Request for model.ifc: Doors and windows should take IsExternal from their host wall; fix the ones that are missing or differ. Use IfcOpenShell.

First a look at what the model holds.

```python
import ifcopenshell
import ifcopenshell.util.element

model = ifcopenshell.open("model.ifc")
print(model.schema)
seen = {}
for e in model.by_type("IfcDoor") + model.by_type("IfcWindow"):
    if not e.FillsVoids:
        continue
    host = e.FillsVoids[0].RelatingOpeningElement.VoidsElements[0].RelatingBuildingElement
    own = ifcopenshell.util.element.get_pset(e, f"Pset_{e.is_a()[3:].removesuffix('StandardCase')}Common", "IsExternal")
    wall = ifcopenshell.util.element.get_pset(host, "Pset_WallCommon", "IsExternal")
    seen[e.is_a(), own, wall] = seen.get((e.is_a(), own, wall), 0) + 1
for (cls, own, wall), count in sorted(seen.items(), key=str):
    print(count, cls, "IsExternal:", own, "| host wall:", wall)
```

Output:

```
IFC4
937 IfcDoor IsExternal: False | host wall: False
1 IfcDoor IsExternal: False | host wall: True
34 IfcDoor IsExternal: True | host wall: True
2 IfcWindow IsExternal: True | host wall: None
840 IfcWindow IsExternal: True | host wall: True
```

```python
import ifcopenshell
import ifcopenshell.api.pset
import ifcopenshell.util.element

model = ifcopenshell.open("model.ifc")

count = 0
for ifc_class, pset_name in (("IfcDoor", "Pset_DoorCommon"), ("IfcWindow", "Pset_WindowCommon")):
    for e in model.by_type(ifc_class):
        if not e.FillsVoids:
            continue
        host = e.FillsVoids[0].RelatingOpeningElement.VoidsElements[0].RelatingBuildingElement
        external = ifcopenshell.util.element.get_pset(host, "Pset_WallCommon", "IsExternal")
        if external is None or ifcopenshell.util.element.get_pset(e, pset_name, "IsExternal") == external:
            continue
        pset = ifcopenshell.api.pset.add_pset(model, product=e, name=pset_name)
        ifcopenshell.api.pset.edit_pset(model, pset=pset, properties={"IsExternal": external})
        count += 1

print(count, "updated")

model.write("model_rev.ifc")
```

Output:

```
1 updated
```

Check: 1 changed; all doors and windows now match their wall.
